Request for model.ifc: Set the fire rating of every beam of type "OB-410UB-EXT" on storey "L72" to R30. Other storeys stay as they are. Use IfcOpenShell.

First a look at what the model holds.

```python
import ifcopenshell
import ifcopenshell.util.element

model = ifcopenshell.open("model.ifc")
print(model.schema)
storey = next(s for s in model.by_type("IfcBuildingStorey") if s.Name == "L72")
beams = [e for e in ifcopenshell.util.element.get_decomposition(storey) if e.is_a("IfcBeam")]
seen = {}
for e in beams:
    element_type = ifcopenshell.util.element.get_type(e)
    key = (element_type.Name if element_type != e and element_type else None, ifcopenshell.util.element.get_pset(e, "Pset_BeamCommon", "FireRating"))
    seen[key] = seen.get(key, 0) + 1
for (name, value), count in sorted(seen.items(), key=str):
    print(count, "x", name, "|", value)
```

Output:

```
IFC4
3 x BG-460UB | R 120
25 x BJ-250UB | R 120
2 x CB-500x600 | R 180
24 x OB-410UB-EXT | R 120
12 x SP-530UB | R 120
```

```python
import ifcopenshell
import ifcopenshell.api.pset
import ifcopenshell.util.element

model = ifcopenshell.open("model.ifc")

storey = next(s for s in model.by_type("IfcBuildingStorey") if s.Name == "L72")
beams = [e for e in ifcopenshell.util.element.get_decomposition(storey) if e.is_a("IfcBeam")]

count = 0
for e in beams:
    element_type = ifcopenshell.util.element.get_type(e)
    if element_type in (None, e) or element_type.Name != "OB-410UB-EXT":
        continue
    found = ifcopenshell.util.element.get_pset(e, "Pset_BeamCommon", should_inherit=False)
    if found:
        pset = model.by_id(found["id"])
        if len(ifcopenshell.util.element.get_elements_by_pset(pset)) > 1:
            pset = ifcopenshell.api.pset.unshare_pset(model, products=[e], pset=pset)[0]
    else:
        pset = ifcopenshell.api.pset.add_pset(model, product=e, name="Pset_BeamCommon")
    ifcopenshell.api.pset.edit_pset(model, pset=pset, properties={"FireRating": "R30"})
    count += 1

print(count, "beams updated")

model.write("model_rev.ifc")
```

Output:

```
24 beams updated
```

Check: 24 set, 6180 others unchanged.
